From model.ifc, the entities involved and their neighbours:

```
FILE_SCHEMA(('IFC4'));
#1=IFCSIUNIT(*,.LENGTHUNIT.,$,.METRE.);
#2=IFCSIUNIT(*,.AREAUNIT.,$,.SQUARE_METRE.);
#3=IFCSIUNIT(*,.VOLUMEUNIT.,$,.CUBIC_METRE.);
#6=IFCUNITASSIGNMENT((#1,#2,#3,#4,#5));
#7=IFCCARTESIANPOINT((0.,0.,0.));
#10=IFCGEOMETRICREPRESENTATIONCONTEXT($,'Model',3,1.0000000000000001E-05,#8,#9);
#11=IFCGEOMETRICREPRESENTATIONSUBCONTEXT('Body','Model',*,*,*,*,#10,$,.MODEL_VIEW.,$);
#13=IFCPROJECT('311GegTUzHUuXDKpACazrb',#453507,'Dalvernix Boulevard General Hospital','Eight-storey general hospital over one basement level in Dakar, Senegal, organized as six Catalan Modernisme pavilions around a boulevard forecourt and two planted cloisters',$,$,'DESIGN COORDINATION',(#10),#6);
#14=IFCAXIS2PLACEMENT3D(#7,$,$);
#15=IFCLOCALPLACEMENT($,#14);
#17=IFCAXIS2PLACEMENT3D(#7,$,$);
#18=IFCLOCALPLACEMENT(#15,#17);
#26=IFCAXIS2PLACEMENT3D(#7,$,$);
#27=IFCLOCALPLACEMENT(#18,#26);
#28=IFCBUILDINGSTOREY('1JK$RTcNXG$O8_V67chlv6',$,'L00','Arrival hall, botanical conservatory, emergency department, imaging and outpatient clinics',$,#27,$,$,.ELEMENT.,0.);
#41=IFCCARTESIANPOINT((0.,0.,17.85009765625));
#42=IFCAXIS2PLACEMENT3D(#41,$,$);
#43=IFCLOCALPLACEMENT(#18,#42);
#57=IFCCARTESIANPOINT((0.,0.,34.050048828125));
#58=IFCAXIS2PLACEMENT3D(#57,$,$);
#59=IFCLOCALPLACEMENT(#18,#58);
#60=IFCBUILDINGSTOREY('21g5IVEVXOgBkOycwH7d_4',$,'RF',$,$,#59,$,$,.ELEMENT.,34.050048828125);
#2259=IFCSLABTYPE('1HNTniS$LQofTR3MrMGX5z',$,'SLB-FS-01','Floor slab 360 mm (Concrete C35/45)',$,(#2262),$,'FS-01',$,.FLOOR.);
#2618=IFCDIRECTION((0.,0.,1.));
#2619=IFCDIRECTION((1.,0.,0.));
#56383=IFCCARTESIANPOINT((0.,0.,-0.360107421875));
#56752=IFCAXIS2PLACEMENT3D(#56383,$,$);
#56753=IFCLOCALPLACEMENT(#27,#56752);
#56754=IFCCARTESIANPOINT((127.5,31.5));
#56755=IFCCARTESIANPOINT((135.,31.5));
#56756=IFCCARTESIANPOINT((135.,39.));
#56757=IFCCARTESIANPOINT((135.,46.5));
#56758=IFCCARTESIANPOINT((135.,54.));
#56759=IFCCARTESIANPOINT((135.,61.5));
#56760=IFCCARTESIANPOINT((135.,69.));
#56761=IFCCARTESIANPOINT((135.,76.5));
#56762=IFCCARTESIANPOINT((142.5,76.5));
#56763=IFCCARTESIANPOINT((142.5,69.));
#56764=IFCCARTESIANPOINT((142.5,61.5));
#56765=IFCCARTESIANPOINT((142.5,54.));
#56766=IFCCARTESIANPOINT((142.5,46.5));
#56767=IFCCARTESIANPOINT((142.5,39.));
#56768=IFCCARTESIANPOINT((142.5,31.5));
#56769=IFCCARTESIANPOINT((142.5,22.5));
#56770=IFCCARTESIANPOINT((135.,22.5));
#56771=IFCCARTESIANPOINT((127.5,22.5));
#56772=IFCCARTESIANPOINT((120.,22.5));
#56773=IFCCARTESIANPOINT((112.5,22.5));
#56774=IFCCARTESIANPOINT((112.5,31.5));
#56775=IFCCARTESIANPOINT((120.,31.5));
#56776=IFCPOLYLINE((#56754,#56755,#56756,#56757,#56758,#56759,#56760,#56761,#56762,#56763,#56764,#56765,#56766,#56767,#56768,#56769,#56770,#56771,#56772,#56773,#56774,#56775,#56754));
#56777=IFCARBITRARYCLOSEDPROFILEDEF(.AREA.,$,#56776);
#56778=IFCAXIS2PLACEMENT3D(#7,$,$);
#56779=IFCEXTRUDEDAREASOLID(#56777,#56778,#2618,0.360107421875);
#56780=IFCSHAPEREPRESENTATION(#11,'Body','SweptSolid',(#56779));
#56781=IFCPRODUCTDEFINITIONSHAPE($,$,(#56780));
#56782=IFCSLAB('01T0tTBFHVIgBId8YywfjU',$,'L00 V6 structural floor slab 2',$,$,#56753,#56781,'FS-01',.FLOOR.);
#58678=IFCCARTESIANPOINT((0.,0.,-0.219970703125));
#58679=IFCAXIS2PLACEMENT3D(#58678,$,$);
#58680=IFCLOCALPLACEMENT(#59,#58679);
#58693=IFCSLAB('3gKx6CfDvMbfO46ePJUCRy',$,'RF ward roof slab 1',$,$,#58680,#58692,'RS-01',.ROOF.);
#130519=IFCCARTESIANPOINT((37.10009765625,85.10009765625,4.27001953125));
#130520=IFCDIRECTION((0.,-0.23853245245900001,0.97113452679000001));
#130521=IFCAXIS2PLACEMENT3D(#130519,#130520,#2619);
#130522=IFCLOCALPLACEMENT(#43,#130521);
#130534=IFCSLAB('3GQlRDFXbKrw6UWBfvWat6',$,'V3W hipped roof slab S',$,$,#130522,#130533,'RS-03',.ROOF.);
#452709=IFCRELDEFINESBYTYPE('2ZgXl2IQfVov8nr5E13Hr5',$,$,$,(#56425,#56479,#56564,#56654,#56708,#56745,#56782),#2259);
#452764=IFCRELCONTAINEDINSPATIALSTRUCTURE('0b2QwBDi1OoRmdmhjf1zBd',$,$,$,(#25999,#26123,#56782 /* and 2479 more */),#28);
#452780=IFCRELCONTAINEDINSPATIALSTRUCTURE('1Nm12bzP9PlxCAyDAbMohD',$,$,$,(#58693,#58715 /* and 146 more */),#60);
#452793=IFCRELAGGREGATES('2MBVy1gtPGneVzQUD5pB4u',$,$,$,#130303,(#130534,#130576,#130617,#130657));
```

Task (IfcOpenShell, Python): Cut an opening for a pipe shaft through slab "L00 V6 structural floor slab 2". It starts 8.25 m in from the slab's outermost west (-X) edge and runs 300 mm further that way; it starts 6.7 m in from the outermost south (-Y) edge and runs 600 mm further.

```python
import numpy as np
import ifcopenshell
import ifcopenshell.api.feature
import ifcopenshell.api.geometry
import ifcopenshell.api.root
import ifcopenshell.geom
import ifcopenshell.util.placement
import ifcopenshell.util.representation
import ifcopenshell.util.shape
import ifcopenshell.util.unit

model = ifcopenshell.open("model.ifc")
unit_scale = ifcopenshell.util.unit.calculate_unit_scale(model)
settings = ifcopenshell.geom.settings()


def volume(element):
    """Net volume in cubic metres, openings subtracted."""
    shape = ifcopenshell.geom.create_shape(settings, element)
    return ifcopenshell.util.shape.get_volume(shape.geometry)


slab = model.by_guid("01T0tTBFHVIgBId8YywfjU")
before = volume(slab)

# Extent in the slab's own axes, in metres. The edges named are its -X and -Y sides.
slab_shape = ifcopenshell.geom.create_shape(settings, slab)
vertices = ifcopenshell.util.shape.get_vertices(slab_shape.geometry)
x_min, y_min, bottom = vertices.min(axis=0)
top = vertices[:, 2].max()

opening = ifcopenshell.api.root.create_entity(model, ifc_class="IfcOpeningElement", name="Pipe shaft opening", predefined_type="OPENING")
context = ifcopenshell.util.representation.get_context(model, "Model", "Body", "MODEL_VIEW")
width, depth = 0.3, 0.6
outline = [(0.0, 0.0), (width, 0.0), (width, depth), (0.0, depth), (0.0, 0.0)]
# Overshoot both faces by 50 mm so the cut is clean.
shape = ifcopenshell.api.geometry.add_slab_representation(
    model, context=context, depth=top - bottom + 0.1, polyline=outline
)
ifcopenshell.api.geometry.assign_representation(model, product=opening, representation=shape)

matrix = ifcopenshell.util.placement.get_local_placement(slab.ObjectPlacement)
matrix[:, 3] = matrix @ np.append(np.array([x_min + 8.25, y_min + 6.7, bottom - 0.05]) / unit_scale, 1.0)
ifcopenshell.api.geometry.edit_object_placement(model, product=opening, matrix=matrix, is_si=False)
ifcopenshell.api.feature.add_feature(model, feature=opening, element=slab)

after = volume(slab)

print(f"slab volume {before:.3f} -> {after:.3f} m3")

model.write("model_edited.ifc")
```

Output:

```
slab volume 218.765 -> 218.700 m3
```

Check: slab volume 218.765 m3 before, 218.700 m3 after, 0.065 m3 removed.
